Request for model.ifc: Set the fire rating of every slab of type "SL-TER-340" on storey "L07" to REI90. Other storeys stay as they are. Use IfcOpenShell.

First a look at what the model holds.

```python
import ifcopenshell
import ifcopenshell.util.element

model = ifcopenshell.open("model.ifc")
print(model.schema)
storey = next(s for s in model.by_type("IfcBuildingStorey") if s.Name == "L07")
slabs = [e for e in ifcopenshell.util.element.get_decomposition(storey) if e.is_a("IfcSlab")]
seen = {}
for e in slabs:
    element_type = ifcopenshell.util.element.get_type(e)
    key = (element_type.Name if element_type != e and element_type else None, ifcopenshell.util.element.get_pset(e, "Pset_SlabCommon", "FireRating"))
    seen[key] = seen.get(key, 0) + 1
for (name, value), count in sorted(seen.items(), key=str):
    print(count, "x", name, "|", value)
```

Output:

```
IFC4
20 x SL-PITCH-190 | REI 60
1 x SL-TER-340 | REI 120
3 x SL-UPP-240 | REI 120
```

```python
import ifcopenshell
import ifcopenshell.api.pset
import ifcopenshell.util.element

model = ifcopenshell.open("model.ifc")

storey = next(s for s in model.by_type("IfcBuildingStorey") if s.Name == "L07")
slabs = [e for e in ifcopenshell.util.element.get_decomposition(storey) if e.is_a("IfcSlab")]

count = 0
for e in slabs:
    element_type = ifcopenshell.util.element.get_type(e)
    if element_type in (None, e) or element_type.Name != "SL-TER-340":
        continue
    # add_pset returns the element's existing set when there is one.
    pset = ifcopenshell.api.pset.add_pset(model, product=e, name="Pset_SlabCommon")
    ifcopenshell.api.pset.edit_pset(model, pset=pset, properties={"FireRating": "REI90"})
    count += 1

print(count, "slabs updated")

model.write("model_rev.ifc")
```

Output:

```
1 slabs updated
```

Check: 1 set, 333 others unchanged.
